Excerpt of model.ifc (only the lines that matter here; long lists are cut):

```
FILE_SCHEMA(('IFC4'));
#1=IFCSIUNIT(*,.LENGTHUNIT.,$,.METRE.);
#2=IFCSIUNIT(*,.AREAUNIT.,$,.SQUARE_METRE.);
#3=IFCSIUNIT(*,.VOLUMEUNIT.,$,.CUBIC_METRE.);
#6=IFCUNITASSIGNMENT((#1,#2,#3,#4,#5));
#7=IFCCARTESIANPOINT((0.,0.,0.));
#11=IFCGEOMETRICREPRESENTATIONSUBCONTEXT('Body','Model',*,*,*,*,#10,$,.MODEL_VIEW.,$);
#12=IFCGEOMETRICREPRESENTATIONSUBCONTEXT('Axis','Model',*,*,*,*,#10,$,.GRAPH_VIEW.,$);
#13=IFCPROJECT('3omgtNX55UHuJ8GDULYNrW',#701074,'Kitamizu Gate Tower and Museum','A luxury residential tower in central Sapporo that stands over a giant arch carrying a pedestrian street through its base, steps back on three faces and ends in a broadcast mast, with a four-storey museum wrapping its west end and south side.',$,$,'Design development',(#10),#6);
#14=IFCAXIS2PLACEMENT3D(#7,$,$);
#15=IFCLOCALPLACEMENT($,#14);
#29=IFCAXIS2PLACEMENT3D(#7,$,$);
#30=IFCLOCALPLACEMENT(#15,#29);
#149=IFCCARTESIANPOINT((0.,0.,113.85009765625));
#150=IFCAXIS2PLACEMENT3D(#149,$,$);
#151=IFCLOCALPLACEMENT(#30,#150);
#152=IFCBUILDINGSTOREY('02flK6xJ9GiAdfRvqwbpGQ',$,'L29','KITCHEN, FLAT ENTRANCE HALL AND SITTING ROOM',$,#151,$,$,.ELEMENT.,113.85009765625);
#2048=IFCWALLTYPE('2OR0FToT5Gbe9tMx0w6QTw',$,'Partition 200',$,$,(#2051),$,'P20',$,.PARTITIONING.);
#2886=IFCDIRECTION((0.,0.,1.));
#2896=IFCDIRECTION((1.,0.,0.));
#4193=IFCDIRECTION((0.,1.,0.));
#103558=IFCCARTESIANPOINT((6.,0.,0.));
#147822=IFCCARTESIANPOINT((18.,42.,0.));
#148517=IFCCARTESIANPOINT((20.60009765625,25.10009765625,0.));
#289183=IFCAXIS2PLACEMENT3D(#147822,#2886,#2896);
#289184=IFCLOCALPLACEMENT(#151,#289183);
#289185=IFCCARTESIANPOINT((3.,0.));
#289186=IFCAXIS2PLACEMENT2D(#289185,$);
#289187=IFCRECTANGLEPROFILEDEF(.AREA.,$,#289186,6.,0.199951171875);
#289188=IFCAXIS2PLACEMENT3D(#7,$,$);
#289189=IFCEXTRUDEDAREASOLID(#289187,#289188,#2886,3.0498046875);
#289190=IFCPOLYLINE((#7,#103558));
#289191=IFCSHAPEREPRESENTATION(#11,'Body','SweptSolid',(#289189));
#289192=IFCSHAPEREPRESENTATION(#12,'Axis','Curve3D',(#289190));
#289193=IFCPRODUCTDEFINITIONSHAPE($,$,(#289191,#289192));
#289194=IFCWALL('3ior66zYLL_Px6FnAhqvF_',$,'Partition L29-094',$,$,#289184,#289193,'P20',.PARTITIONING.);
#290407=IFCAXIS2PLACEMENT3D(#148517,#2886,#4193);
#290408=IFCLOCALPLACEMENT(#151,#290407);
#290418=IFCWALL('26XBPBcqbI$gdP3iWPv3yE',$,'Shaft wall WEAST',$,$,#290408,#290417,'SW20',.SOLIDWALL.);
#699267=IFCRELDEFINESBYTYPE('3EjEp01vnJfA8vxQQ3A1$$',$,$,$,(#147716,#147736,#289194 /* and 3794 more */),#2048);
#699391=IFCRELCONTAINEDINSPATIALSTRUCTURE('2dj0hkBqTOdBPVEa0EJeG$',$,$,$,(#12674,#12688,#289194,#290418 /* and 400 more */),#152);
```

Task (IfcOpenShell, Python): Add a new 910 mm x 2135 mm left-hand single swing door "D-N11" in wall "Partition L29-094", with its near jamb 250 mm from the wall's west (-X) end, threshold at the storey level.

```python
import numpy as np
import ifcopenshell
import ifcopenshell.api.feature
import ifcopenshell.api.geometry
import ifcopenshell.api.root
import ifcopenshell.api.spatial
import ifcopenshell.geom
import ifcopenshell.util.element
import ifcopenshell.util.placement
import ifcopenshell.util.representation
import ifcopenshell.util.shape
import ifcopenshell.util.unit

model = ifcopenshell.open("model.ifc")
unit_scale = ifcopenshell.util.unit.calculate_unit_scale(model)
settings = ifcopenshell.geom.settings()


def volume(element):
    """Net volume in cubic metres, openings subtracted."""
    shape = ifcopenshell.geom.create_shape(settings, element)
    return ifcopenshell.util.shape.get_volume(shape.geometry)


wall = model.by_id(289194)
storey = ifcopenshell.util.element.get_container(wall, ifc_class="IfcBuildingStorey")
context = ifcopenshell.util.representation.get_context(model, "Model", "Body", "MODEL_VIEW")
before = volume(wall)

width, height, from_end, sill = 0.91, 2.135, 0.25, 0.0  # metres

# The wall runs along its own X axis, and the end named is its -X end.
wall_shape = ifcopenshell.geom.create_shape(settings, wall)
x, y, z = ifcopenshell.util.shape.get_vertices(wall_shape.geometry).T
start = x.min() + from_end
face, thickness = float(y.min()), float(y.max() - y.min())
wall_matrix = ifcopenshell.util.placement.get_local_placement(wall.ObjectPlacement)
level = ifcopenshell.util.placement.get_local_placement(storey.ObjectPlacement)[2, 3]


def in_wall(x, y):
    """Placement at x, y metres in the wall's axes, at sill height."""
    matrix = wall_matrix.copy()
    matrix[:, 3] = wall_matrix @ np.array([x / unit_scale, y / unit_scale, 0.0, 1.0])
    matrix[2, 3] = level + sill / unit_scale
    return matrix


# Opening: a box that overshoots both wall faces by 50 mm.
opening = ifcopenshell.api.root.create_entity(model, ifc_class="IfcOpeningElement", predefined_type="OPENING")
box = ifcopenshell.api.geometry.add_wall_representation(
    model, context=context, length=width, height=height, thickness=thickness + 0.1
)
ifcopenshell.api.geometry.assign_representation(model, product=opening, representation=box)
ifcopenshell.api.geometry.edit_object_placement(model, product=opening, matrix=in_wall(start, face - 0.05), is_si=False)
ifcopenshell.api.feature.add_feature(model, feature=opening, element=wall)

door = ifcopenshell.api.root.create_entity(model, ifc_class="IfcDoor", name="D-N11", predefined_type="DOOR")
door.OverallWidth, door.OverallHeight = width / unit_scale, height / unit_scale
door.OperationType = "SINGLE_SWING_LEFT"
body = ifcopenshell.api.geometry.add_door_representation(
    model,
    context=context,
    overall_width=door.OverallWidth,
    overall_height=door.OverallHeight,
    operation_type="SINGLE_SWING_LEFT",
    lining_properties={"LiningDepth": thickness / unit_scale, "ThresholdDepth": thickness / unit_scale},
)
ifcopenshell.api.geometry.assign_representation(model, product=door, representation=body)
ifcopenshell.api.spatial.assign_container(model, products=[door], relating_structure=storey)
ifcopenshell.api.feature.add_filling(model, opening=opening, element=door)

# The lining spans the wall, so the door starts at the wall face.
ifcopenshell.api.geometry.edit_object_placement(model, product=door, matrix=in_wall(start, face), is_si=False)

after = volume(wall)

print(f"wall volume {before:.3f} -> {after:.3f} m3")

model.write("model_v2.ifc")
```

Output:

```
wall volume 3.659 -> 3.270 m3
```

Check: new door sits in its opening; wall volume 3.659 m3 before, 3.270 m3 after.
